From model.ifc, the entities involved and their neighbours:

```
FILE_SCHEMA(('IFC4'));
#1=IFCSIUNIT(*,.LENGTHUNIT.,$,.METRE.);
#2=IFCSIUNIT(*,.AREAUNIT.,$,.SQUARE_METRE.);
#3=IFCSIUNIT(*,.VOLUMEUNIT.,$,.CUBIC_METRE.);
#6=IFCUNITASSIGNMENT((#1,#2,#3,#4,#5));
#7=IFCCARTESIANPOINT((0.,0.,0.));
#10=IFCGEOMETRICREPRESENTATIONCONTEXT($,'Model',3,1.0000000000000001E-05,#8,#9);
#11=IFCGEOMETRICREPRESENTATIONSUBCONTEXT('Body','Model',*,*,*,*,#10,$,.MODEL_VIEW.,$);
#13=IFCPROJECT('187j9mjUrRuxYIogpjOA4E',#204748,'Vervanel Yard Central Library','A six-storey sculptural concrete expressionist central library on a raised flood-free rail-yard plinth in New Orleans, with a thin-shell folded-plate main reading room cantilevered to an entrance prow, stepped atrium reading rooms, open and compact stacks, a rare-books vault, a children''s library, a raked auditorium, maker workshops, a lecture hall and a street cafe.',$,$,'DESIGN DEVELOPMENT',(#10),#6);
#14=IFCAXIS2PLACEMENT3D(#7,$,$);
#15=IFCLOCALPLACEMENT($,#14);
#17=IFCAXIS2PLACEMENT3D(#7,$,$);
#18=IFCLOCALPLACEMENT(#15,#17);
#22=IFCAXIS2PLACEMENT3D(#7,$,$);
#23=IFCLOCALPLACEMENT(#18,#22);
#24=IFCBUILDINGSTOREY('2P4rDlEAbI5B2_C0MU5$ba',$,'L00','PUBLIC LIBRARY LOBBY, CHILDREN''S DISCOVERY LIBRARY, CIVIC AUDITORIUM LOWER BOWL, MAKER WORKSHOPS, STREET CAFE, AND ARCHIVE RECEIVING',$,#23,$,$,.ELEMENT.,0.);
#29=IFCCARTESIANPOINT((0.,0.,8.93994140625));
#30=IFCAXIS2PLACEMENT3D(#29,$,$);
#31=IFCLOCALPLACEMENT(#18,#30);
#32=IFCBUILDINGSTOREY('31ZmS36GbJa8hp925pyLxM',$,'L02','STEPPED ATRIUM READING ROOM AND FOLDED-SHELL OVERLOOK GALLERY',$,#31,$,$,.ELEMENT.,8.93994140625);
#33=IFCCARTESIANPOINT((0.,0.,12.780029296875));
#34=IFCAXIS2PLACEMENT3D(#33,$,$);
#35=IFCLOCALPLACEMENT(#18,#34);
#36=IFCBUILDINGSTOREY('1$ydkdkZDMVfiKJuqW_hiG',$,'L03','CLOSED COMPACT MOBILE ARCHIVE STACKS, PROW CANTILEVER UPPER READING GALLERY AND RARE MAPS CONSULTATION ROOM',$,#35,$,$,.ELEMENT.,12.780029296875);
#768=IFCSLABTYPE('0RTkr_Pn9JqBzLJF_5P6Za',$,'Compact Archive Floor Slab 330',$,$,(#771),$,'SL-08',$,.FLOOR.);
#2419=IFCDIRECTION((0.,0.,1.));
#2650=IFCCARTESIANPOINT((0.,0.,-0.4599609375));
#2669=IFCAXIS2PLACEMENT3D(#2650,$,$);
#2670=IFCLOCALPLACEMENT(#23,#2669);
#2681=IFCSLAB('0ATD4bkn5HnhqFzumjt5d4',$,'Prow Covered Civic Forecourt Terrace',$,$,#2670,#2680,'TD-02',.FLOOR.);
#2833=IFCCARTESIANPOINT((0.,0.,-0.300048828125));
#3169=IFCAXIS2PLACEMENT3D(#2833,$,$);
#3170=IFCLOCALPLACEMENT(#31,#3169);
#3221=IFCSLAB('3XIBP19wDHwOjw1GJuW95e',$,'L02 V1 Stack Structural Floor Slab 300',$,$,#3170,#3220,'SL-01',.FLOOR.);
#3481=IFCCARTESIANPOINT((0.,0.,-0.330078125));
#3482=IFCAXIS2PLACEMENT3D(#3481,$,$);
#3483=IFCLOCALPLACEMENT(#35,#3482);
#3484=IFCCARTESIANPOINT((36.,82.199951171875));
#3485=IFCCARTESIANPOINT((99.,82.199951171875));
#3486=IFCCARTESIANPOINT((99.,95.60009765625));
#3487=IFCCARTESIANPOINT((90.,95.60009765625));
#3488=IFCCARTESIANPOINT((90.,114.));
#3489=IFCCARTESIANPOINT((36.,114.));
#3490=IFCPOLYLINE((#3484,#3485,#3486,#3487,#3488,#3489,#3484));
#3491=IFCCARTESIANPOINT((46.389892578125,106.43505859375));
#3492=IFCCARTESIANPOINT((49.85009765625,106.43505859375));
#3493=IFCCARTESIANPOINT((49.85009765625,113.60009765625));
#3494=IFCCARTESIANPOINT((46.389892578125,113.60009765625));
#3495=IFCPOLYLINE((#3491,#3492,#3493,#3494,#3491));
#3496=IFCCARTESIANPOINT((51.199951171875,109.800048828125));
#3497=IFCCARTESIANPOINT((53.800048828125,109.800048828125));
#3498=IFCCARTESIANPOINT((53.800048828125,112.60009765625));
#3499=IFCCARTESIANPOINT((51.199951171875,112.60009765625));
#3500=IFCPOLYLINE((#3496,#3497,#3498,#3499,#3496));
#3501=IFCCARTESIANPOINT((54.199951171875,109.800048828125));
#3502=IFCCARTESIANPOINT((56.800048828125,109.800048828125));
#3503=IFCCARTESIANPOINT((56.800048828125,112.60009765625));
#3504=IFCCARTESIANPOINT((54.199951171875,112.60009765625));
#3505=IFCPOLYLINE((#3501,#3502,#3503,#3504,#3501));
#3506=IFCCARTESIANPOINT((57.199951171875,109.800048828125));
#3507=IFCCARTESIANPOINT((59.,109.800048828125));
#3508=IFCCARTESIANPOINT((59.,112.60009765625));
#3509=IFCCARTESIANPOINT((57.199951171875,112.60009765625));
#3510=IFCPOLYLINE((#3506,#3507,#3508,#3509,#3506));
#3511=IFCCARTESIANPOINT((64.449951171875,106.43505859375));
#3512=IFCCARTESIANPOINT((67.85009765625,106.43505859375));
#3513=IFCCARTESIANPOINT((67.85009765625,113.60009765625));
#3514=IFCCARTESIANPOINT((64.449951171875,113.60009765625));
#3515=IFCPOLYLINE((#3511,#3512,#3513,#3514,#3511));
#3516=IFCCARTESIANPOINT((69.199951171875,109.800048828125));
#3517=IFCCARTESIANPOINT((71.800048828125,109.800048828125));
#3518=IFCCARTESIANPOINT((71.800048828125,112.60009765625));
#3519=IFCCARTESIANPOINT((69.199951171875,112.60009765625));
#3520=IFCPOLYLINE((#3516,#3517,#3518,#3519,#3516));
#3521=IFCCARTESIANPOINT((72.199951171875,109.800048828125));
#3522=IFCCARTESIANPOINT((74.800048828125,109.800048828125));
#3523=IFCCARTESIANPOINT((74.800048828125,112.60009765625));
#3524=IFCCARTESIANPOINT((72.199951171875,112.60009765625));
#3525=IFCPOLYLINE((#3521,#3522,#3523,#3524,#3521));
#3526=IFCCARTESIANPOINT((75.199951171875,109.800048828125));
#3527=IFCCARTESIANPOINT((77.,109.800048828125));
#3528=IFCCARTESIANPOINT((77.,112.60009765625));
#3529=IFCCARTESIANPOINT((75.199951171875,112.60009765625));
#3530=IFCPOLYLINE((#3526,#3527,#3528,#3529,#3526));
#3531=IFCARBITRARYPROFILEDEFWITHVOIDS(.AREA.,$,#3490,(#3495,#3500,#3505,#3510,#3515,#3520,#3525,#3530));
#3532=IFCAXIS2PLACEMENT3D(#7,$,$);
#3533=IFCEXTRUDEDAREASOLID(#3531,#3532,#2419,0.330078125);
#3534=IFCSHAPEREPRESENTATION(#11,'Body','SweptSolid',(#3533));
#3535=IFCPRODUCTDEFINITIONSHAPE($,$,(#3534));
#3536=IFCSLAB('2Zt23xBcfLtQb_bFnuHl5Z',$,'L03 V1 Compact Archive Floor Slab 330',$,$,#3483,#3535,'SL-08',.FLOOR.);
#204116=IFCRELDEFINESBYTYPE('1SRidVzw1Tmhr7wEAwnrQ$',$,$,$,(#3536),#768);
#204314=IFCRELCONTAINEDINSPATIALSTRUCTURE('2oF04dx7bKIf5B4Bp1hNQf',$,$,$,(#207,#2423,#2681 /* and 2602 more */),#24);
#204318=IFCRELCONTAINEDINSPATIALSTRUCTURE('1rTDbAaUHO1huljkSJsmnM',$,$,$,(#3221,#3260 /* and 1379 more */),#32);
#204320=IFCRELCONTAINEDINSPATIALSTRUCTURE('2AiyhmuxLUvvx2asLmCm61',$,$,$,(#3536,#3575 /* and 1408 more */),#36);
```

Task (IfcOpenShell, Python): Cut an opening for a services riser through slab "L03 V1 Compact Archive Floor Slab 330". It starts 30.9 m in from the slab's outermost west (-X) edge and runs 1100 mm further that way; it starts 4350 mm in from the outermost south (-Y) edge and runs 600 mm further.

```python
import numpy as np
import ifcopenshell
import ifcopenshell.api.feature
import ifcopenshell.api.geometry
import ifcopenshell.api.root
import ifcopenshell.geom
import ifcopenshell.util.placement
import ifcopenshell.util.representation
import ifcopenshell.util.shape
import ifcopenshell.util.unit

model = ifcopenshell.open("model.ifc")
unit_scale = ifcopenshell.util.unit.calculate_unit_scale(model)
settings = ifcopenshell.geom.settings()


def volume(element):
    """Net volume in cubic metres, openings subtracted."""
    shape = ifcopenshell.geom.create_shape(settings, element)
    return ifcopenshell.util.shape.get_volume(shape.geometry)


slab = model.by_guid("2Zt23xBcfLtQb_bFnuHl5Z")
before = volume(slab)

# Extent in the slab's own axes, in metres. The edges named are its -X and -Y sides.
slab_shape = ifcopenshell.geom.create_shape(settings, slab)
vertices = ifcopenshell.util.shape.get_vertices(slab_shape.geometry)
x_min, y_min, bottom = vertices.min(axis=0)
top = vertices[:, 2].max()

opening = ifcopenshell.api.root.create_entity(model, ifc_class="IfcOpeningElement", name="Services riser opening", predefined_type="OPENING")
context = ifcopenshell.util.representation.get_context(model, "Model", "Body", "MODEL_VIEW")
width, depth = 1.1, 0.6
outline = [(0.0, 0.0), (width, 0.0), (width, depth), (0.0, depth), (0.0, 0.0)]
# Overshoot both faces by 50 mm so the cut is clean.
shape = ifcopenshell.api.geometry.add_slab_representation(
    model, context=context, depth=top - bottom + 0.1, polyline=outline
)
ifcopenshell.api.geometry.assign_representation(model, product=opening, representation=shape)

matrix = ifcopenshell.util.placement.get_local_placement(slab.ObjectPlacement)
matrix[:, 3] = matrix @ np.append(np.array([x_min + 30.9, y_min + 4.35, bottom - 0.05]) / unit_scale, 1.0)
ifcopenshell.api.geometry.edit_object_placement(model, product=opening, matrix=matrix, is_si=False)
ifcopenshell.api.feature.add_feature(model, feature=opening, element=slab)

after = volume(slab)

print(f"slab volume {before:.3f} -> {after:.3f} m3")

model.write("model_rev.ifc")
```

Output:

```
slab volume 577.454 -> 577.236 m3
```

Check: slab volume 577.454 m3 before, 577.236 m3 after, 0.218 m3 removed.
